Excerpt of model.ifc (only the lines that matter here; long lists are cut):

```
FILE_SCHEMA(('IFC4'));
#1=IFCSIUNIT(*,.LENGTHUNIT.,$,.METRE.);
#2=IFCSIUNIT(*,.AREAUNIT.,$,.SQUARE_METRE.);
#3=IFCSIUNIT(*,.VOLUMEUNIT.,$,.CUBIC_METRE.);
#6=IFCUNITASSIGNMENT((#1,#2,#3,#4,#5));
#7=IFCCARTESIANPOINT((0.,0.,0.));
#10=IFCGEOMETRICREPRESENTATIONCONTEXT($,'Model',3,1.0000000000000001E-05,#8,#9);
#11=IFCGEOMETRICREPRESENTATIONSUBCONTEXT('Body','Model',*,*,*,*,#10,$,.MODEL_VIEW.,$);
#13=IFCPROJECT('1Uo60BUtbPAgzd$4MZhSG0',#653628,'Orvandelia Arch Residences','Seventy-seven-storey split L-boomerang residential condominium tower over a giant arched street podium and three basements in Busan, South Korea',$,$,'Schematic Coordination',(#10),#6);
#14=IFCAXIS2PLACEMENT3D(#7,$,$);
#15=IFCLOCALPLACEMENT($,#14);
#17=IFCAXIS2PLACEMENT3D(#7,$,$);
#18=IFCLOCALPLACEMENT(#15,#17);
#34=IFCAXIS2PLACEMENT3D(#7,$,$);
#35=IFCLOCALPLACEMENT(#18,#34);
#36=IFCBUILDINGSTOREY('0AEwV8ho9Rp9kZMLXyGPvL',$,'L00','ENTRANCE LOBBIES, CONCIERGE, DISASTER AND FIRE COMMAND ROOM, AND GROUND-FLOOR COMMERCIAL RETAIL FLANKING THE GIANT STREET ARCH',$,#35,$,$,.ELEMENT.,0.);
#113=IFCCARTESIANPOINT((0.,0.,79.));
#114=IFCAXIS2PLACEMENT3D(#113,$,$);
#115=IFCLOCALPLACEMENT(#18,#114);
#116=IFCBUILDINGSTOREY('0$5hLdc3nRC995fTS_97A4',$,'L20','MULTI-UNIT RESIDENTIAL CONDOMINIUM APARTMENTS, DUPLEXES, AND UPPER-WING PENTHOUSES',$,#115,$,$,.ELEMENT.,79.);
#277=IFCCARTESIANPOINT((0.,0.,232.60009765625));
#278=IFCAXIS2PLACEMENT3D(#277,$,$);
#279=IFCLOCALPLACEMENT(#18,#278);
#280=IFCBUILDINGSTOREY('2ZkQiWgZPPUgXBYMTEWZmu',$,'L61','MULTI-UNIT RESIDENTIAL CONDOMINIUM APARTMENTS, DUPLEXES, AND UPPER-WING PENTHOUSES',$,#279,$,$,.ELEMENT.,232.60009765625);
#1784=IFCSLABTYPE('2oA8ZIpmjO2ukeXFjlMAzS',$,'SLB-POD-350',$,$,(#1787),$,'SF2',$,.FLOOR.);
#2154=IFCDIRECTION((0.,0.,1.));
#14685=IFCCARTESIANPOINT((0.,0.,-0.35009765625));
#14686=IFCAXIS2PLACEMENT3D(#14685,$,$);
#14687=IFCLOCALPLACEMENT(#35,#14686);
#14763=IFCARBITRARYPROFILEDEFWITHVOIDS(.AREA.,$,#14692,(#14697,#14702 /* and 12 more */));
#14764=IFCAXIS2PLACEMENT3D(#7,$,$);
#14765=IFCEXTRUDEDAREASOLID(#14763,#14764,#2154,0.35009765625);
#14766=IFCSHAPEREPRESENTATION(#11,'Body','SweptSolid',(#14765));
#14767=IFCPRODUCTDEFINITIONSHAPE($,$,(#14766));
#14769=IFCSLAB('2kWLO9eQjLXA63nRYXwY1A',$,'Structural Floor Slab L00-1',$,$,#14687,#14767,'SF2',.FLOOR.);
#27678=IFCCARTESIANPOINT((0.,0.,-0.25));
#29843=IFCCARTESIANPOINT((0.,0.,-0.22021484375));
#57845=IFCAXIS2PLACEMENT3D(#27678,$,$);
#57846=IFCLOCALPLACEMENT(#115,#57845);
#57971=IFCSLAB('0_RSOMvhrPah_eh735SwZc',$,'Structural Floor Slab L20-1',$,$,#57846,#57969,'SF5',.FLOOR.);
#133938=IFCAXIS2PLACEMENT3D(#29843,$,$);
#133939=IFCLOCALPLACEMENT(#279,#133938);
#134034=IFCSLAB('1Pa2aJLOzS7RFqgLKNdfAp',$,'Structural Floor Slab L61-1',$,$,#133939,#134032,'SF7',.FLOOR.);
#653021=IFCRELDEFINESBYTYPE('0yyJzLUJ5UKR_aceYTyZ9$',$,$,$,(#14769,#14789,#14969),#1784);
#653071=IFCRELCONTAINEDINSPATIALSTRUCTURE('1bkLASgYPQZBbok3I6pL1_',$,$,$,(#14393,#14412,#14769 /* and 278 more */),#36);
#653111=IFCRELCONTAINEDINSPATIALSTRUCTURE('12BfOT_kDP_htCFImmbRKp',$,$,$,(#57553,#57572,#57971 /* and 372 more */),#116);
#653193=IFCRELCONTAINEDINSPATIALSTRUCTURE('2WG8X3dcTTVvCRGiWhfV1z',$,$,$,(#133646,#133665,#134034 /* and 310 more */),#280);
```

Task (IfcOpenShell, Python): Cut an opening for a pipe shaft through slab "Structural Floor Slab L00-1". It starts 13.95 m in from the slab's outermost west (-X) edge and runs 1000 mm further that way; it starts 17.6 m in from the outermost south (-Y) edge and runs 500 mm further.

```python
import numpy as np
import ifcopenshell
import ifcopenshell.api.feature
import ifcopenshell.api.geometry
import ifcopenshell.api.root
import ifcopenshell.geom
import ifcopenshell.util.placement
import ifcopenshell.util.representation
import ifcopenshell.util.shape
import ifcopenshell.util.unit

model = ifcopenshell.open("model.ifc")
unit_scale = ifcopenshell.util.unit.calculate_unit_scale(model)
settings = ifcopenshell.geom.settings()


def volume(element):
    """Net volume in cubic metres, openings subtracted."""
    shape = ifcopenshell.geom.create_shape(settings, element)
    return ifcopenshell.util.shape.get_volume(shape.geometry)


slab = model.by_guid("2kWLO9eQjLXA63nRYXwY1A")
before = volume(slab)

# Extent in the slab's own axes, in metres. The edges named are its -X and -Y sides.
slab_shape = ifcopenshell.geom.create_shape(settings, slab)
vertices = ifcopenshell.util.shape.get_vertices(slab_shape.geometry)
x_min, y_min, bottom = vertices.min(axis=0)
top = vertices[:, 2].max()

opening = ifcopenshell.api.root.create_entity(model, ifc_class="IfcOpeningElement", name="Pipe shaft opening", predefined_type="OPENING")
context = ifcopenshell.util.representation.get_context(model, "Model", "Body", "MODEL_VIEW")
width, depth = 1, 0.5
outline = [(0.0, 0.0), (width, 0.0), (width, depth), (0.0, depth), (0.0, 0.0)]
# Overshoot both faces by 50 mm so the cut is clean.
shape = ifcopenshell.api.geometry.add_slab_representation(
    model, context=context, depth=top - bottom + 0.1, polyline=outline
)
ifcopenshell.api.geometry.assign_representation(model, product=opening, representation=shape)

matrix = ifcopenshell.util.placement.get_local_placement(slab.ObjectPlacement)
matrix[:, 3] = matrix @ np.append(np.array([x_min + 13.95, y_min + 17.6, bottom - 0.05]) / unit_scale, 1.0)
ifcopenshell.api.geometry.edit_object_placement(model, product=opening, matrix=matrix, is_si=False)
ifcopenshell.api.feature.add_feature(model, feature=opening, element=slab)

after = volume(slab)

print(f"slab volume {before:.3f} -> {after:.3f} m3")

model.write("model_edited.ifc")
```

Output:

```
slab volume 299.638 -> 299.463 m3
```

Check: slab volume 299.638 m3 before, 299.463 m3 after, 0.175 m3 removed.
